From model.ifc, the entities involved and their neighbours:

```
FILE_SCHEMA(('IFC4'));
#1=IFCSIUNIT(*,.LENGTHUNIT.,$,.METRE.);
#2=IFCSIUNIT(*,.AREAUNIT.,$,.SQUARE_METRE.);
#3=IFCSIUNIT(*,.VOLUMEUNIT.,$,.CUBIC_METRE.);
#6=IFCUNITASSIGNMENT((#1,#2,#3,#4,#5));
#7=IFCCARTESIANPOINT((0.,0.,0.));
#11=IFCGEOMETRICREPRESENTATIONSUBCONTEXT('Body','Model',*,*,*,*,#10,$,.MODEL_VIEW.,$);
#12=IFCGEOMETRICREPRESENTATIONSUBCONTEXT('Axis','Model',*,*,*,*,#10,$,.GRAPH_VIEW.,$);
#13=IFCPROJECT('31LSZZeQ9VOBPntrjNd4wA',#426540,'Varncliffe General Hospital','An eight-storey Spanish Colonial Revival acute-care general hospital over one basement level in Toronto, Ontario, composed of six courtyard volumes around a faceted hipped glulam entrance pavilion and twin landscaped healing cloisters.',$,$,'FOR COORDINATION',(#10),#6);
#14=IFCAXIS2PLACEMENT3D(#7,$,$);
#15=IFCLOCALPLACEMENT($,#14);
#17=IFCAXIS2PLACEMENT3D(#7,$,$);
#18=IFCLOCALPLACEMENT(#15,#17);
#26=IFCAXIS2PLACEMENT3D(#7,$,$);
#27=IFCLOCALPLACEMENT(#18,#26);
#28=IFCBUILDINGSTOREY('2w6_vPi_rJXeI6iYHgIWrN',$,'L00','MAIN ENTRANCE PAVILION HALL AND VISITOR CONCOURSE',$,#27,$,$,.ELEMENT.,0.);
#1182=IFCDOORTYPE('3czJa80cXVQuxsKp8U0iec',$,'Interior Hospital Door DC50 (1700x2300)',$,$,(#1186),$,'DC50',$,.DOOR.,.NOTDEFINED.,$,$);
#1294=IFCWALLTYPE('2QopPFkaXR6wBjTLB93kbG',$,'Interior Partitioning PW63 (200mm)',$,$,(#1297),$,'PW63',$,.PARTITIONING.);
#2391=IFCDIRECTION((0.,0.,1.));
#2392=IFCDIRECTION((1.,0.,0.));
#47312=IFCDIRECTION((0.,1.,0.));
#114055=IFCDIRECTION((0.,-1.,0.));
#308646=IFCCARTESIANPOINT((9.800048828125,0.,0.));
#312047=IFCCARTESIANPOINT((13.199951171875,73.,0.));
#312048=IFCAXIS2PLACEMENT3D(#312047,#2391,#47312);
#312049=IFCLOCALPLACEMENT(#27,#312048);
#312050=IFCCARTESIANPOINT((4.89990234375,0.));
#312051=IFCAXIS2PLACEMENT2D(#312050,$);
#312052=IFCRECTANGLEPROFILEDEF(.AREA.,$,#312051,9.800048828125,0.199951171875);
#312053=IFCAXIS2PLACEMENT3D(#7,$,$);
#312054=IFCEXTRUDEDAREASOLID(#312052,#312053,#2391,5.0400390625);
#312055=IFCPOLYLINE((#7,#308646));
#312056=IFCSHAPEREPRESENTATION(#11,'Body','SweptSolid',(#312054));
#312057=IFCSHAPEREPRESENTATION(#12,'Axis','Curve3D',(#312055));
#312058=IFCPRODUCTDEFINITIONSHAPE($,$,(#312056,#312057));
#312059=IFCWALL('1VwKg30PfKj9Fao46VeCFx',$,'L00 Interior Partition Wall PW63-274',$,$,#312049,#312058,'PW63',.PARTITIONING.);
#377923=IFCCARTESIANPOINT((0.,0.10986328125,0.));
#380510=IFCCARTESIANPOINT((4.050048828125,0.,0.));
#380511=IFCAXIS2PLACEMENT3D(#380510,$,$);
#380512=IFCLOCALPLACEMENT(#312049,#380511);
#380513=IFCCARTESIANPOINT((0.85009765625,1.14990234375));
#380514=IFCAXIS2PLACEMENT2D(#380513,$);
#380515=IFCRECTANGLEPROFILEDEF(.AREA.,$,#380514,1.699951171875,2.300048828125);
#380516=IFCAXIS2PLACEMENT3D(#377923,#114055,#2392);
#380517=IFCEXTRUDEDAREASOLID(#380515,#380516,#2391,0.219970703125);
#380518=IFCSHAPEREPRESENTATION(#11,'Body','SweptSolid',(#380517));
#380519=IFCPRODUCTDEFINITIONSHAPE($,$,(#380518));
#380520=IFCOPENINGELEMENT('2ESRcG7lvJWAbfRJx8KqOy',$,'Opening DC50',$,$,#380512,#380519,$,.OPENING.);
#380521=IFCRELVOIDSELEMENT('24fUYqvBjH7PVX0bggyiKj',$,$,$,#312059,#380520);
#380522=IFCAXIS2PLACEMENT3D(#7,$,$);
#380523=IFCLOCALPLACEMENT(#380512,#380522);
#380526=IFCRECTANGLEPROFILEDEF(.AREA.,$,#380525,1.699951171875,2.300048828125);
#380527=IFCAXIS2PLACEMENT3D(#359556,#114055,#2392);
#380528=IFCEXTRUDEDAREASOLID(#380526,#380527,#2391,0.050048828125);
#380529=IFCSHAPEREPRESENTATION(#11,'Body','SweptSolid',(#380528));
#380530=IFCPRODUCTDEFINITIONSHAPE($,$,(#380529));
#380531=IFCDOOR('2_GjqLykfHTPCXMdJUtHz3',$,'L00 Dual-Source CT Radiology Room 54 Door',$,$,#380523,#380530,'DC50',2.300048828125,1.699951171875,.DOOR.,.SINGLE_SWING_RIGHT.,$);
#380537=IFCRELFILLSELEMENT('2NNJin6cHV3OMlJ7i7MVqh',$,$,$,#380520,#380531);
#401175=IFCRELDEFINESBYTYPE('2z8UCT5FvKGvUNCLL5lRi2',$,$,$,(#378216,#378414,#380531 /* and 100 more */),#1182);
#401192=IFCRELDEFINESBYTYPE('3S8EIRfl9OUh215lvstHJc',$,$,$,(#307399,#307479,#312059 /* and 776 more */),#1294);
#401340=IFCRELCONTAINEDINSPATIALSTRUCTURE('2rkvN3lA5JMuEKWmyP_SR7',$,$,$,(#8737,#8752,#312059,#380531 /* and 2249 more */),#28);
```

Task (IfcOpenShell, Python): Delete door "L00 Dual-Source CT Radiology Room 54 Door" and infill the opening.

```python
import ifcopenshell
import ifcopenshell.api.feature
import ifcopenshell.api.root
import ifcopenshell.geom
import ifcopenshell.util.shape

model = ifcopenshell.open("model.ifc")
settings = ifcopenshell.geom.settings()


def volume(element):
    """Net volume in cubic metres, openings subtracted."""
    shape = ifcopenshell.geom.create_shape(settings, element)
    return ifcopenshell.util.shape.get_volume(shape.geometry)


door = model.by_guid("2_GjqLykfHTPCXMdJUtHz3")
opening = door.FillsVoids[0].RelatingOpeningElement
wall = opening.VoidsElements[0].RelatingBuildingElement
before = volume(wall)

ifcopenshell.api.root.remove_product(model, product=door)
ifcopenshell.api.feature.remove_feature(model, feature=opening)

after = volume(wall)

print(f"wall volume {before:.3f} -> {after:.3f} m3")

model.write("model_updated.ifc")
```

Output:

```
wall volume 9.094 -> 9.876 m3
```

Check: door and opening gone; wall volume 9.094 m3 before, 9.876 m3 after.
